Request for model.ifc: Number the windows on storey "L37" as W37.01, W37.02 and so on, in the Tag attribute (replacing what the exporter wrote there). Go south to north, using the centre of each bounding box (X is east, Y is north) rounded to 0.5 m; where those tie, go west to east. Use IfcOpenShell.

First a look at what the model holds.

```python
import ifcopenshell
import ifcopenshell.util.element
import ifcopenshell.util.placement

model = ifcopenshell.open("model.ifc")
print(model.schema)
storey = next(s for s in model.by_type("IfcBuildingStorey") if s.Name == "L37")
windows = [e for e in ifcopenshell.util.element.get_decomposition(storey) if e.is_a("IfcWindow")]
for e in sorted(windows, key=lambda e: e.id()):
    origin = ifcopenshell.util.placement.get_local_placement(e.ObjectPlacement)[:3, 3]
    print(e.id(), e.Tag, e.Name, origin.round(2) + 0.0, sep=" | ")
```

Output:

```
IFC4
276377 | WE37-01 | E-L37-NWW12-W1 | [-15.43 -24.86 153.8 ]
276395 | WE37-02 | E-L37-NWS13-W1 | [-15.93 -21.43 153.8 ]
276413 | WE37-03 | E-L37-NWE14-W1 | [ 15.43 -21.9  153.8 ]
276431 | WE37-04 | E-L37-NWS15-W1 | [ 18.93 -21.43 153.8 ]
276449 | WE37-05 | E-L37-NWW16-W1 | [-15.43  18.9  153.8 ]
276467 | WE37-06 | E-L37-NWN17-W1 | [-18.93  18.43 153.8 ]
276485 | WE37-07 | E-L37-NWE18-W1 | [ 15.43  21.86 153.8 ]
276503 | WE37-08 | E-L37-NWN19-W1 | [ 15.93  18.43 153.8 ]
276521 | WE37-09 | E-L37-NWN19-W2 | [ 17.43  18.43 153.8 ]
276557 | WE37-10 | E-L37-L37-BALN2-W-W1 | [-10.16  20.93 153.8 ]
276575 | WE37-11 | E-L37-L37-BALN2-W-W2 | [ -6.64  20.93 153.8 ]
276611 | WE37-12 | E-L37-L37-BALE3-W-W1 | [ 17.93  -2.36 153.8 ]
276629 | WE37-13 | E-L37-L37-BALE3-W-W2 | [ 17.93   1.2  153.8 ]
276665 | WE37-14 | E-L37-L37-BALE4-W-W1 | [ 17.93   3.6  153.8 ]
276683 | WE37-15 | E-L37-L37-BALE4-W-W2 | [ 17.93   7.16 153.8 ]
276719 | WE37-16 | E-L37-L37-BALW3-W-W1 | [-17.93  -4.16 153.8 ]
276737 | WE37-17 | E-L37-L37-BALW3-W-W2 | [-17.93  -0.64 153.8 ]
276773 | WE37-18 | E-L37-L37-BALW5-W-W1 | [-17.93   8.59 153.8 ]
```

```python
import ifcopenshell
import ifcopenshell.geom
import ifcopenshell.util.element
import ifcopenshell.util.shape

model = ifcopenshell.open("model.ifc")
settings = ifcopenshell.geom.settings()
settings.set("use-world-coords", True)


def centre(element):
    shape = ifcopenshell.geom.create_shape(settings, element)
    return ifcopenshell.util.shape.get_bbox_centroid(shape.geometry)


storey = next(s for s in model.by_type("IfcBuildingStorey") if s.Name == "L37")
windows = [e for e in ifcopenshell.util.element.get_decomposition(storey) if e.is_a("IfcWindow")]

# Insertion points can sit at a corner or the storey origin, so sort by the geometry (in metres).
centres = {e: centre(e) for e in windows}
windows.sort(key=lambda e: (round(centres[e][1] / 0.5), centres[e][0]))

for i, e in enumerate(windows, start=1):
    number = f"W37.{i:02d}"
    e.Tag = number
    print(e.id(), number)

model.write("model_edited.ifc")
```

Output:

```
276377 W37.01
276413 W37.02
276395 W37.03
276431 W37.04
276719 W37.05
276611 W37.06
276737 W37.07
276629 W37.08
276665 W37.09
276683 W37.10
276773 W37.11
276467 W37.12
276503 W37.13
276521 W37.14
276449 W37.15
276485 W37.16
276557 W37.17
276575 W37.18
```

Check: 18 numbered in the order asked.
